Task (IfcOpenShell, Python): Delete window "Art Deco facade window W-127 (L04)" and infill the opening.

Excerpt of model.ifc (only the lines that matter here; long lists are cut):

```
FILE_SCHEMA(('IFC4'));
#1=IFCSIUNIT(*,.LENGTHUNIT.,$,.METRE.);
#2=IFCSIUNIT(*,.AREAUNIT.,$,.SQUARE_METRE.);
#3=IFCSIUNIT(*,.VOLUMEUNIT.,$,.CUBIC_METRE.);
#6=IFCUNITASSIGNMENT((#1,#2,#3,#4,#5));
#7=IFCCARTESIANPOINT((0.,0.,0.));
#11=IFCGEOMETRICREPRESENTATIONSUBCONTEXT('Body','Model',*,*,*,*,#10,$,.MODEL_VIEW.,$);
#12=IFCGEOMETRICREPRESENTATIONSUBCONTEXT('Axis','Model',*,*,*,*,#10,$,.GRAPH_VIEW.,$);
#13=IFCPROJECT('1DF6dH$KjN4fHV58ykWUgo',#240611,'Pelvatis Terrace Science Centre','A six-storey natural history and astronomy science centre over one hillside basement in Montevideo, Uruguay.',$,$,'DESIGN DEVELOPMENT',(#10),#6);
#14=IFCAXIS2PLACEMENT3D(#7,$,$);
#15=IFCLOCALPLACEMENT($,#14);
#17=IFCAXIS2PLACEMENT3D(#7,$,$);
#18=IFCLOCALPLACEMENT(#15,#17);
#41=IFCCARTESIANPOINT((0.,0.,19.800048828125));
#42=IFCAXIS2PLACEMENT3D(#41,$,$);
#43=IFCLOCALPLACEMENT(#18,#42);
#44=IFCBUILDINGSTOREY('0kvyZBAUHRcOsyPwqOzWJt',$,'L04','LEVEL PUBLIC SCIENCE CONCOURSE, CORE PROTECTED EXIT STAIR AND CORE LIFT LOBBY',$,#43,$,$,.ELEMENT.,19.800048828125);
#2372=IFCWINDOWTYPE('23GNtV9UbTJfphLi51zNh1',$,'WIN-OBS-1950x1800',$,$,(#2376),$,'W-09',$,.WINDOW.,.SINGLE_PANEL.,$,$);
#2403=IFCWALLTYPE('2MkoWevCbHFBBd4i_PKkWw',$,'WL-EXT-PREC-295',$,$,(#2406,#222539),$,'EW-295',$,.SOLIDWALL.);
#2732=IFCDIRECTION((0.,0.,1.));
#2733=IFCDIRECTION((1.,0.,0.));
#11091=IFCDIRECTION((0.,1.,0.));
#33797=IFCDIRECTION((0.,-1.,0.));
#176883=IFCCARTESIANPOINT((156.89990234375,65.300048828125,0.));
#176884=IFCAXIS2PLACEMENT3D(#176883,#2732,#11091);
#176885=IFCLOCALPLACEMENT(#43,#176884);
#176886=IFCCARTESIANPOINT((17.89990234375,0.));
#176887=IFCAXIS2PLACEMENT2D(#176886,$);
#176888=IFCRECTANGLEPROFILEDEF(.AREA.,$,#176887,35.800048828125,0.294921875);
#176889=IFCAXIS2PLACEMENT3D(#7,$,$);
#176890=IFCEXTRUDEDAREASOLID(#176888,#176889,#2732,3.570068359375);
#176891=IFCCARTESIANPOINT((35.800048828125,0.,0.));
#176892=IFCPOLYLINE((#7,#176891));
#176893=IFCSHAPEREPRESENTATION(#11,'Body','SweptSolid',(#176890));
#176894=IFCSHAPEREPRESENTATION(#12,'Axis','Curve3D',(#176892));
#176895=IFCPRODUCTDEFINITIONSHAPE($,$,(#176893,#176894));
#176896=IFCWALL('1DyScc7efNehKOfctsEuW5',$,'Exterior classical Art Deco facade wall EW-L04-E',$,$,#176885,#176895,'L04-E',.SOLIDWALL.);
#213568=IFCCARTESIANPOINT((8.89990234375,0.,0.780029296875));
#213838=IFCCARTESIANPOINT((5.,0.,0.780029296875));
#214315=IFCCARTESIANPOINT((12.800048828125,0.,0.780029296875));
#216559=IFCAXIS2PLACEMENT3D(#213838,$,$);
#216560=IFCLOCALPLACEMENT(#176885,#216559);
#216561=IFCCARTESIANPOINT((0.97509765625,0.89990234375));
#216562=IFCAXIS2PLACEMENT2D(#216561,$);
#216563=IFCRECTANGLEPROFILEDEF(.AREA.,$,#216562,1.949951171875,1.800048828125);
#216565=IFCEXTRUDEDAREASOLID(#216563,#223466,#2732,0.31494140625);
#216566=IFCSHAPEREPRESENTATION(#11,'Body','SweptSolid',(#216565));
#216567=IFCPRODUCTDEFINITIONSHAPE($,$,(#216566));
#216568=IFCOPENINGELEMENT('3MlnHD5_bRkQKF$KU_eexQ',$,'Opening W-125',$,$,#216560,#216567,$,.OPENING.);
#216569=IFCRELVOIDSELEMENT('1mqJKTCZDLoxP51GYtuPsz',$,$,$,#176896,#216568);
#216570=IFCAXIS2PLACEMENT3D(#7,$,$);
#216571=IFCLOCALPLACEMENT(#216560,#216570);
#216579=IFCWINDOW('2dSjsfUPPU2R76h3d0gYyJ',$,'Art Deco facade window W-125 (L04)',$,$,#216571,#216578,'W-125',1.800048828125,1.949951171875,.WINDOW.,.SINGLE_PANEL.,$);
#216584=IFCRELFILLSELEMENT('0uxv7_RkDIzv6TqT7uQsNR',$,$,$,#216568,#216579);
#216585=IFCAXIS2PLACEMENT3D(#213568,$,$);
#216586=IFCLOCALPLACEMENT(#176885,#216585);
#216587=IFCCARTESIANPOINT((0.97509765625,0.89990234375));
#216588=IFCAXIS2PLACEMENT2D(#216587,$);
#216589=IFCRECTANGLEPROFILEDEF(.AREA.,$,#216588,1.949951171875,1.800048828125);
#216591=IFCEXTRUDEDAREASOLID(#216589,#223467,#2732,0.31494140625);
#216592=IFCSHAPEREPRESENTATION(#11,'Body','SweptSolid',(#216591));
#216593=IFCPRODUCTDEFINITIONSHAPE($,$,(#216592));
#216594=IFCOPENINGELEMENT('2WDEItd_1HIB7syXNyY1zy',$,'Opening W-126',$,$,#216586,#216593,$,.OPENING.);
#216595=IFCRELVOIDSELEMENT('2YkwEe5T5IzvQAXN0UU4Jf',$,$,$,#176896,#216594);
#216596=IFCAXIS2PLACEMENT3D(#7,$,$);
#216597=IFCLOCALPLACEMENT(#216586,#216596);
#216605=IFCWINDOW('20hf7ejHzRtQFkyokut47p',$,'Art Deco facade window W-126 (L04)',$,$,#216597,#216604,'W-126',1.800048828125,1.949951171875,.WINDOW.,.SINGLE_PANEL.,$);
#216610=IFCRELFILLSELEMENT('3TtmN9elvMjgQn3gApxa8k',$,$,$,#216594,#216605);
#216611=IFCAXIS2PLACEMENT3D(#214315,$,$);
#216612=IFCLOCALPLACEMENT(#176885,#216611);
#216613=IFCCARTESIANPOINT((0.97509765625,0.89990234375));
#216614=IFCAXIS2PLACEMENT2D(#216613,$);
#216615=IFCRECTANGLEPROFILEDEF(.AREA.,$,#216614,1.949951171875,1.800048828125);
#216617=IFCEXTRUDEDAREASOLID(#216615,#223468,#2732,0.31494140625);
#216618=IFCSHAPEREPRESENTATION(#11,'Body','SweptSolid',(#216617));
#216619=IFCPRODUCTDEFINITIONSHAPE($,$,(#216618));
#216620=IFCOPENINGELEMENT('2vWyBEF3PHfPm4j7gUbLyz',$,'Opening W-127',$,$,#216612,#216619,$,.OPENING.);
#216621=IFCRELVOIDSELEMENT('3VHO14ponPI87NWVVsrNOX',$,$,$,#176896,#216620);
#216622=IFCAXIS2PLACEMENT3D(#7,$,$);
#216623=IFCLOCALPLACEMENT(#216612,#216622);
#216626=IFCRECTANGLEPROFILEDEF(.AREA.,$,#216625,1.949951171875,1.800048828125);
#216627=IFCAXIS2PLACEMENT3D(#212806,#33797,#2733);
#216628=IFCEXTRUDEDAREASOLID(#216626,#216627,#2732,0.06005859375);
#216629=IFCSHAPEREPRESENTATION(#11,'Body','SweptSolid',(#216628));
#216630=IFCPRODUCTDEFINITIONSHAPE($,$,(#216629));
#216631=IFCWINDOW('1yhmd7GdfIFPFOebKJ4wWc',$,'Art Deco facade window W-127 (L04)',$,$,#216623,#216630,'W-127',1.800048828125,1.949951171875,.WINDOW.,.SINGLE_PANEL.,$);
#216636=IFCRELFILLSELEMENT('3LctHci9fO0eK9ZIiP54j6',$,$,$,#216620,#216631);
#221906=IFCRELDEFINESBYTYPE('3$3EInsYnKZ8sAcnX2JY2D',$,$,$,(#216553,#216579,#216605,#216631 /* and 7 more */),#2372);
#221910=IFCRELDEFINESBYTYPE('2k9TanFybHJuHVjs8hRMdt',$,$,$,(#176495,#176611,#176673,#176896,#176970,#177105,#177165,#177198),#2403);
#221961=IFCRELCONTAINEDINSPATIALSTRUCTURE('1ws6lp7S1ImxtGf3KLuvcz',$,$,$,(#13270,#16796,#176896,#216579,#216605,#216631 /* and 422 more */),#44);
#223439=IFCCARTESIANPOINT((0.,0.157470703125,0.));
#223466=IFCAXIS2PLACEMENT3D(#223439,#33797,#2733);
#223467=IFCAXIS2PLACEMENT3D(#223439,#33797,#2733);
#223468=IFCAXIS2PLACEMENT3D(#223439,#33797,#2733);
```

```python
import ifcopenshell
import ifcopenshell.api.feature
import ifcopenshell.api.root
import ifcopenshell.geom
import ifcopenshell.util.shape

model = ifcopenshell.open("model.ifc")
settings = ifcopenshell.geom.settings()


def volume(element):
    """Net volume in cubic metres, openings subtracted."""
    shape = ifcopenshell.geom.create_shape(settings, element)
    return ifcopenshell.util.shape.get_volume(shape.geometry)


window = model.by_guid("1yhmd7GdfIFPFOebKJ4wWc")
opening = window.FillsVoids[0].RelatingOpeningElement
wall = opening.VoidsElements[0].RelatingBuildingElement
before = volume(wall)

ifcopenshell.api.root.remove_product(model, product=window)
ifcopenshell.api.feature.remove_feature(model, feature=opening)

after = volume(wall)

print(f"wall volume {before:.3f} -> {after:.3f} m3")

model.write("model_updated.ifc")
```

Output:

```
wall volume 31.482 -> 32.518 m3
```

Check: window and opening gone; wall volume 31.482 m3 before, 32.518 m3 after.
